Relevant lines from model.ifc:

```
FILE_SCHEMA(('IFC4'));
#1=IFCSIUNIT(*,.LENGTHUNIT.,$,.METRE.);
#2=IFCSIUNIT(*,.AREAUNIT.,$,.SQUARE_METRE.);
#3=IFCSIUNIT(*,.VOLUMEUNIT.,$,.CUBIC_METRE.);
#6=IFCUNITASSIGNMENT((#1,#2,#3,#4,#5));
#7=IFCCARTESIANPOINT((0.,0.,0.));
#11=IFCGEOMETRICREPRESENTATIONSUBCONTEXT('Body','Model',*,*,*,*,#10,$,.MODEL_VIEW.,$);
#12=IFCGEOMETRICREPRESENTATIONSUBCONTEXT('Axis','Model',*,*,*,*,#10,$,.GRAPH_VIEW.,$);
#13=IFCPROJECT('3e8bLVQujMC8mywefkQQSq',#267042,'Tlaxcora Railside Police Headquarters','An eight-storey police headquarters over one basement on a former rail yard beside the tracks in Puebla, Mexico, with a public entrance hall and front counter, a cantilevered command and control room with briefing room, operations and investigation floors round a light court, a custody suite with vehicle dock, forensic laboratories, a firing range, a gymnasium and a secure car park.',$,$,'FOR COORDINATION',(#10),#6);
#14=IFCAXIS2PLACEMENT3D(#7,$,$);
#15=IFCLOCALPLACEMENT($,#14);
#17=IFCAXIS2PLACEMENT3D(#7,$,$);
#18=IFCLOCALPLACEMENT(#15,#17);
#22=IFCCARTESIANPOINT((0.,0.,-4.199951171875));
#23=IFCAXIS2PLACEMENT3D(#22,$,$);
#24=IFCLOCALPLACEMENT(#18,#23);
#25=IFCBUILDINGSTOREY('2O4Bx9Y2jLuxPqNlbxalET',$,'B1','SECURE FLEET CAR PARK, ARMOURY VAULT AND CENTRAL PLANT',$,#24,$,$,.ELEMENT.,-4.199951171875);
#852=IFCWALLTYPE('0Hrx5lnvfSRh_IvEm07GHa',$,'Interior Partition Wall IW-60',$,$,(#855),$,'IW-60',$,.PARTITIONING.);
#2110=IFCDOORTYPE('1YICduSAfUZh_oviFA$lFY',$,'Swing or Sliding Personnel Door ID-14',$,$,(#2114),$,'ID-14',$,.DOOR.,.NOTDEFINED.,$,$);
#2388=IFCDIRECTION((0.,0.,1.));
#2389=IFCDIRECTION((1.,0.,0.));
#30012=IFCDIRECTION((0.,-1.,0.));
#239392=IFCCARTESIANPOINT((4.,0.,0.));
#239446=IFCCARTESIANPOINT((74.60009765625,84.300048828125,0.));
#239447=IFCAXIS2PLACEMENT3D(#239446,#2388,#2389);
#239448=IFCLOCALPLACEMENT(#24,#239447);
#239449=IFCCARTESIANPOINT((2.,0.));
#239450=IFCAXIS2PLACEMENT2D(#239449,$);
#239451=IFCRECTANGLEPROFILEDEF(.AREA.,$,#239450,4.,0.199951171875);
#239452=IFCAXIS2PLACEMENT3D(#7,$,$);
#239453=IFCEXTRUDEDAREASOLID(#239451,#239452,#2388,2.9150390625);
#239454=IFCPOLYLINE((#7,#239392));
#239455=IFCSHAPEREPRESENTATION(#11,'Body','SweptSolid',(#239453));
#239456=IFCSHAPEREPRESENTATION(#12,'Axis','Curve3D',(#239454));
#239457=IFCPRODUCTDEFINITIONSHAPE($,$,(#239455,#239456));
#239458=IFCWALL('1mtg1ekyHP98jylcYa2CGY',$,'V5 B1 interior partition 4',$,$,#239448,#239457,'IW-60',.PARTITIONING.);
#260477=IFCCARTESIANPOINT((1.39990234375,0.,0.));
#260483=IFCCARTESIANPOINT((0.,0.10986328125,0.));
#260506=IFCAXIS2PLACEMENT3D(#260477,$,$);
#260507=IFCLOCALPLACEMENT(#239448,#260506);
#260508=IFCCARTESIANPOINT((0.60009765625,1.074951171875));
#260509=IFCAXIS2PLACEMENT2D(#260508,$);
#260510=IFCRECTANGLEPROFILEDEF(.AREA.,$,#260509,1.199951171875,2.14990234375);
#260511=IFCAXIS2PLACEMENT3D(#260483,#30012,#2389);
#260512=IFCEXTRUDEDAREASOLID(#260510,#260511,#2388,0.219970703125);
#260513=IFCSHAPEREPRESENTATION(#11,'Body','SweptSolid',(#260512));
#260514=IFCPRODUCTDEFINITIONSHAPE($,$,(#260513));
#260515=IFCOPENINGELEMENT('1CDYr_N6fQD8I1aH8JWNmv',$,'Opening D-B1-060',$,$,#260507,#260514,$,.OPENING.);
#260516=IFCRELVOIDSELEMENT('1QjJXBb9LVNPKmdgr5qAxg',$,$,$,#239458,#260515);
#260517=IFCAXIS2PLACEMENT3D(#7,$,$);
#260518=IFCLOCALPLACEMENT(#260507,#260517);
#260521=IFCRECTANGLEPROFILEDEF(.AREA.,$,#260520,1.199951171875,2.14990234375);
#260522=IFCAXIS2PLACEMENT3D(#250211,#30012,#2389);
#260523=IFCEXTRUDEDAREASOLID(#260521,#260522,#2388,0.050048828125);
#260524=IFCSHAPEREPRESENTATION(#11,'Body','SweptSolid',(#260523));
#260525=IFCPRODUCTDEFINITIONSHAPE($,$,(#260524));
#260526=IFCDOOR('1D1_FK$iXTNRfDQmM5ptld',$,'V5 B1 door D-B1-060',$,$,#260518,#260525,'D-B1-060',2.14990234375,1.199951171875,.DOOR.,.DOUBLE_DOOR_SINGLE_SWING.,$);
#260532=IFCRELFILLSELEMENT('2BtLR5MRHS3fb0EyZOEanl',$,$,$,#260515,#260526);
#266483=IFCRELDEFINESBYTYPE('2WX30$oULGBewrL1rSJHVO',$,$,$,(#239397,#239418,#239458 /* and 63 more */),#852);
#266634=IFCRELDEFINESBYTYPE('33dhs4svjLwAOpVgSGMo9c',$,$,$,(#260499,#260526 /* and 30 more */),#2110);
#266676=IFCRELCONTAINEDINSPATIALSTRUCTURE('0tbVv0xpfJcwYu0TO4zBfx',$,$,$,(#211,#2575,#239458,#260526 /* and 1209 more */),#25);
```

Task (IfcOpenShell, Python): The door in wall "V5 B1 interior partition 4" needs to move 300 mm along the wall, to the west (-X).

```python
import ifcopenshell
import ifcopenshell.api.geometry
import ifcopenshell.util.placement
import ifcopenshell.util.unit

model = ifcopenshell.open("model.ifc")
unit_scale = ifcopenshell.util.unit.calculate_unit_scale(model)

door = model.by_guid("1D1_FK$iXTNRfDQmM5ptld")
opening = door.FillsVoids[0].RelatingOpeningElement
wall = opening.VoidsElements[0].RelatingBuildingElement

wall_matrix = ifcopenshell.util.placement.get_local_placement(wall.ObjectPlacement)
shift = wall_matrix[:3, 0] * -0.3 / unit_scale
before = ifcopenshell.util.placement.get_local_placement(door.ObjectPlacement)[:3, 3].copy()

# The door is placed relative to its opening, so it follows when the opening moves.
matrix = ifcopenshell.util.placement.get_local_placement(opening.ObjectPlacement)
matrix[:3, 3] += shift
ifcopenshell.api.geometry.edit_object_placement(
    model, product=opening, matrix=matrix, is_si=False, should_transform_children=True
)

after = ifcopenshell.util.placement.get_local_placement(door.ObjectPlacement)[:3, 3]
print("door moved by", (after - before).round(3) + 0.0)

model.write("model_updated.ifc")
```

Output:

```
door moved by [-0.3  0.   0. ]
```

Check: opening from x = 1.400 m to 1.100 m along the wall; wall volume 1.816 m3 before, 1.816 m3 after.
